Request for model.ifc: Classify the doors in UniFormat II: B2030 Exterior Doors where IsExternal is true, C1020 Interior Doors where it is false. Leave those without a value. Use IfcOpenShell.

First a look at what the model holds.

```python
import ifcopenshell
import ifcopenshell.util.element

model = ifcopenshell.open("model.ifc")
print(model.schema)
print("classifications:", [c.Name for c in model.by_type("IfcClassification")])
values = [ifcopenshell.util.element.get_pset(e, "Pset_DoorCommon", "IsExternal") for e in model.by_type("IfcDoor")]
for value in (True, False, None):
    print("IsExternal", value, values.count(value))
```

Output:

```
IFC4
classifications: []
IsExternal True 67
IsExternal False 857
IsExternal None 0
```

```python
import ifcopenshell
import ifcopenshell.api.classification
import ifcopenshell.util.element

model = ifcopenshell.open("model.ifc")

system = ifcopenshell.api.classification.add_classification(model, classification="UniFormat II")

doors = model.by_type("IfcDoor")
external = {e: ifcopenshell.util.element.get_pset(e, "Pset_DoorCommon", "IsExternal") for e in doors}
for flag, code, name in ((True, "B2030", "Exterior Doors"), (False, "C1020", "Interior Doors")):
    products = [e for e in doors if external[e] is flag]
    ifcopenshell.api.classification.add_reference(
        model, products=products, classification=system, identification=code, name=name
    )
    print(code, len(products))

model.write("model_edited.ifc")
```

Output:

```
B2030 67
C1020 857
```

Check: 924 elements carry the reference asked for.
